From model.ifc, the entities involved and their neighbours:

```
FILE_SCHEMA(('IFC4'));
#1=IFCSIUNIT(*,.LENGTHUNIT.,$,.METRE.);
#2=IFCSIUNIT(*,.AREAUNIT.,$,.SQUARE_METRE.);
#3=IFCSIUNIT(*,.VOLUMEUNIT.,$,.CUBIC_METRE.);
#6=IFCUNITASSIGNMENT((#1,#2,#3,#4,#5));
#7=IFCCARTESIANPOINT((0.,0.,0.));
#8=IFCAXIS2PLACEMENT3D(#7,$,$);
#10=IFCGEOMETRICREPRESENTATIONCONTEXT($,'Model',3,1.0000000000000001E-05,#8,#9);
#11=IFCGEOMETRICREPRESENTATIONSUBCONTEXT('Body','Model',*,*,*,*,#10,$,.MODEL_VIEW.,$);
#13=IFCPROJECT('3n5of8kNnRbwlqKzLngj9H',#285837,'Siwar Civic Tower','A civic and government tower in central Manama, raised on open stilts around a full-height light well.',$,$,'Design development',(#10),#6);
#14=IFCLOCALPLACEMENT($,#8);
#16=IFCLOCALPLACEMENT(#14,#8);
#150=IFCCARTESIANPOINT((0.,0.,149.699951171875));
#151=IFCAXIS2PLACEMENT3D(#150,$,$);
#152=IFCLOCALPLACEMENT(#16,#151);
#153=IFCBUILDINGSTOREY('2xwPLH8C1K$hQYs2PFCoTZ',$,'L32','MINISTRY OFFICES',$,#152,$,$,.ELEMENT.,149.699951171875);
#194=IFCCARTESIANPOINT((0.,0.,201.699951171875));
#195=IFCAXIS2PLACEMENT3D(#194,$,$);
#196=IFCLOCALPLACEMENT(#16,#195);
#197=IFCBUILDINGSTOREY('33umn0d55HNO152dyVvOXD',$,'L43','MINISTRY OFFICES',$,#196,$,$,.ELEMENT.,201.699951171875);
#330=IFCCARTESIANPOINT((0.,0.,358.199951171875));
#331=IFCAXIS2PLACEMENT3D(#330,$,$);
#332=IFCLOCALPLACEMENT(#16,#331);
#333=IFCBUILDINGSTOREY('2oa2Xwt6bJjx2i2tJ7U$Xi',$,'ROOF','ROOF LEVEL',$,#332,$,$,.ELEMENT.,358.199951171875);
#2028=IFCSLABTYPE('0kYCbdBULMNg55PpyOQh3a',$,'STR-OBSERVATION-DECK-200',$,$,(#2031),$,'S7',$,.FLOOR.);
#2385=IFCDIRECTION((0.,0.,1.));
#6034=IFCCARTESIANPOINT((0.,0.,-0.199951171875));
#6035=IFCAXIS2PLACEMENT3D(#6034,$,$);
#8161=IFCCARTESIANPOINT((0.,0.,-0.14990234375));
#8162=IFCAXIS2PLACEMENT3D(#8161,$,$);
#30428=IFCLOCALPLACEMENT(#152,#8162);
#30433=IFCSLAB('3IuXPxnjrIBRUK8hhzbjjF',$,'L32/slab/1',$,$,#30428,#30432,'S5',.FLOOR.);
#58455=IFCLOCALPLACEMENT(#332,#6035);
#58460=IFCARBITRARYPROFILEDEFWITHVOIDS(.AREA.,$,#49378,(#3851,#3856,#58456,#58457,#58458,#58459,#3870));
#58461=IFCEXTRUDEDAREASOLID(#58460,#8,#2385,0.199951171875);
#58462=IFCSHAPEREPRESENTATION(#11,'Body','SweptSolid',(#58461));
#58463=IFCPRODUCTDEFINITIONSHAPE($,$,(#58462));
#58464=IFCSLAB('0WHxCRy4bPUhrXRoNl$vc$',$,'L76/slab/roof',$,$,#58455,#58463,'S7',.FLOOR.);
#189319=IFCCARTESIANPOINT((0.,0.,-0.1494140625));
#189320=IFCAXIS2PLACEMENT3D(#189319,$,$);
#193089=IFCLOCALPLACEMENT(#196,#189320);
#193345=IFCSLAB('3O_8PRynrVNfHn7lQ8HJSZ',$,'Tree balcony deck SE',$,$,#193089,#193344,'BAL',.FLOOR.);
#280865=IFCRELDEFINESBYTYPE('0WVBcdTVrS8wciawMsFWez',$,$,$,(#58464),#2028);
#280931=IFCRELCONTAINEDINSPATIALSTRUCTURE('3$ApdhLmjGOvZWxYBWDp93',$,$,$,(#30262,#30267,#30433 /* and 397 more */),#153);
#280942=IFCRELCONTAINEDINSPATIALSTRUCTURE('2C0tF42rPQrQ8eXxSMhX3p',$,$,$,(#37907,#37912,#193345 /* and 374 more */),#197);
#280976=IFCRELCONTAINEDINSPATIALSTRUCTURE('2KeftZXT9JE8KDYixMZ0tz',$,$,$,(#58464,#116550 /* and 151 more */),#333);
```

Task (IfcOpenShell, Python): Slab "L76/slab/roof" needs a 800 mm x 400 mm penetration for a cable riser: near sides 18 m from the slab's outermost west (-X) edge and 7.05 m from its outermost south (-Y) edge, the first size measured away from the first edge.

```python
import numpy as np
import ifcopenshell
import ifcopenshell.api.feature
import ifcopenshell.api.geometry
import ifcopenshell.api.root
import ifcopenshell.geom
import ifcopenshell.util.placement
import ifcopenshell.util.representation
import ifcopenshell.util.shape
import ifcopenshell.util.unit

model = ifcopenshell.open("model.ifc")
unit_scale = ifcopenshell.util.unit.calculate_unit_scale(model)
settings = ifcopenshell.geom.settings()


def volume(element):
    """Net volume in cubic metres, openings subtracted."""
    shape = ifcopenshell.geom.create_shape(settings, element)
    return ifcopenshell.util.shape.get_volume(shape.geometry)


slab = model.by_guid("0WHxCRy4bPUhrXRoNl$vc$")
before = volume(slab)

# Extent in the slab's own axes, in metres. The edges named are its -X and -Y sides.
slab_shape = ifcopenshell.geom.create_shape(settings, slab)
vertices = ifcopenshell.util.shape.get_vertices(slab_shape.geometry)
x_min, y_min, bottom = vertices.min(axis=0)
top = vertices[:, 2].max()

opening = ifcopenshell.api.root.create_entity(model, ifc_class="IfcOpeningElement", name="Cable riser opening", predefined_type="OPENING")
context = ifcopenshell.util.representation.get_context(model, "Model", "Body", "MODEL_VIEW")
width, depth = 0.8, 0.4
outline = [(0.0, 0.0), (width, 0.0), (width, depth), (0.0, depth), (0.0, 0.0)]
# Overshoot both faces by 50 mm so the cut is clean.
shape = ifcopenshell.api.geometry.add_slab_representation(
    model, context=context, depth=top - bottom + 0.1, polyline=outline
)
ifcopenshell.api.geometry.assign_representation(model, product=opening, representation=shape)

matrix = ifcopenshell.util.placement.get_local_placement(slab.ObjectPlacement)
matrix[:, 3] = matrix @ np.append(np.array([x_min + 18, y_min + 7.05, bottom - 0.05]) / unit_scale, 1.0)
ifcopenshell.api.geometry.edit_object_placement(model, product=opening, matrix=matrix, is_si=False)
ifcopenshell.api.feature.add_feature(model, feature=opening, element=slab)

after = volume(slab)

print(f"slab volume {before:.3f} -> {after:.3f} m3")

model.write("model_updated.ifc")
```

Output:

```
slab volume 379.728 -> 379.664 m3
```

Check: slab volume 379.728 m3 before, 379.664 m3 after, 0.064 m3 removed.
